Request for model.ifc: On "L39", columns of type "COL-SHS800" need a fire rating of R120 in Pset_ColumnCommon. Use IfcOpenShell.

First a look at what the model holds.

```python
import ifcopenshell
import ifcopenshell.util.element

model = ifcopenshell.open("model.ifc")
print(model.schema)
storey = next(s for s in model.by_type("IfcBuildingStorey") if s.Name == "L39")
columns = [e for e in ifcopenshell.util.element.get_decomposition(storey) if e.is_a("IfcColumn")]
seen = {}
for e in columns:
    element_type = ifcopenshell.util.element.get_type(e)
    key = (element_type.Name if element_type != e and element_type else None, ifcopenshell.util.element.get_pset(e, "Pset_ColumnCommon", "FireRating"))
    seen[key] = seen.get(key, 0) + 1
for (name, value), count in sorted(seen.items(), key=str):
    print(count, "x", name, "|", value)
```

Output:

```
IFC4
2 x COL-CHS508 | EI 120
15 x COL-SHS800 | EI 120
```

```python
import ifcopenshell
import ifcopenshell.api.pset
import ifcopenshell.util.element

model = ifcopenshell.open("model.ifc")

storey = next(s for s in model.by_type("IfcBuildingStorey") if s.Name == "L39")
columns = [e for e in ifcopenshell.util.element.get_decomposition(storey) if e.is_a("IfcColumn")]

count = 0
for e in columns:
    element_type = ifcopenshell.util.element.get_type(e)
    if element_type in (None, e) or element_type.Name != "COL-SHS800":
        continue
    # add_pset returns the element's existing set when there is one.
    pset = ifcopenshell.api.pset.add_pset(model, product=e, name="Pset_ColumnCommon")
    ifcopenshell.api.pset.edit_pset(model, pset=pset, properties={"FireRating": "R120"})
    count += 1

print(count, "columns updated")

model.write("model_updated.ifc")
```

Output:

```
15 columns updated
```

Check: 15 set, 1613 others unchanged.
